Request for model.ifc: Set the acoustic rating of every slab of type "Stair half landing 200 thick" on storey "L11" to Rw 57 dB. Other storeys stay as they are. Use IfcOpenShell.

First a look at what the model holds.

```python
import ifcopenshell
import ifcopenshell.util.element

model = ifcopenshell.open("model.ifc")
print(model.schema)
storey = next(s for s in model.by_type("IfcBuildingStorey") if s.Name == "L11")
slabs = [e for e in ifcopenshell.util.element.get_decomposition(storey) if e.is_a("IfcSlab")]
seen = {}
for e in slabs:
    element_type = ifcopenshell.util.element.get_type(e)
    key = (element_type.Name if element_type != e and element_type else None, ifcopenshell.util.element.get_pset(e, "Pset_SlabCommon", "AcousticRating"))
    seen[key] = seen.get(key, 0) + 1
for (name, value), count in sorted(seen.items(), key=str):
    print(count, "x", name, "|", value)
```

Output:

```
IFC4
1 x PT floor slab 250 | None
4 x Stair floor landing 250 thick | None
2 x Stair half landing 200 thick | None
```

```python
import ifcopenshell
import ifcopenshell.api.pset
import ifcopenshell.util.element

model = ifcopenshell.open("model.ifc")

storey = next(s for s in model.by_type("IfcBuildingStorey") if s.Name == "L11")
slabs = [e for e in ifcopenshell.util.element.get_decomposition(storey) if e.is_a("IfcSlab")]

count = 0
for e in slabs:
    element_type = ifcopenshell.util.element.get_type(e)
    if element_type in (None, e) or element_type.Name != "Stair half landing 200 thick":
        continue
    # add_pset returns the element's existing set when there is one.
    pset = ifcopenshell.api.pset.add_pset(model, product=e, name="Pset_SlabCommon")
    ifcopenshell.api.pset.edit_pset(model, pset=pset, properties={"AcousticRating": "Rw 57 dB"})
    count += 1

print(count, "slabs updated")

model.write("model_v2.ifc")
```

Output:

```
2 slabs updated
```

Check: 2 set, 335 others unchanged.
